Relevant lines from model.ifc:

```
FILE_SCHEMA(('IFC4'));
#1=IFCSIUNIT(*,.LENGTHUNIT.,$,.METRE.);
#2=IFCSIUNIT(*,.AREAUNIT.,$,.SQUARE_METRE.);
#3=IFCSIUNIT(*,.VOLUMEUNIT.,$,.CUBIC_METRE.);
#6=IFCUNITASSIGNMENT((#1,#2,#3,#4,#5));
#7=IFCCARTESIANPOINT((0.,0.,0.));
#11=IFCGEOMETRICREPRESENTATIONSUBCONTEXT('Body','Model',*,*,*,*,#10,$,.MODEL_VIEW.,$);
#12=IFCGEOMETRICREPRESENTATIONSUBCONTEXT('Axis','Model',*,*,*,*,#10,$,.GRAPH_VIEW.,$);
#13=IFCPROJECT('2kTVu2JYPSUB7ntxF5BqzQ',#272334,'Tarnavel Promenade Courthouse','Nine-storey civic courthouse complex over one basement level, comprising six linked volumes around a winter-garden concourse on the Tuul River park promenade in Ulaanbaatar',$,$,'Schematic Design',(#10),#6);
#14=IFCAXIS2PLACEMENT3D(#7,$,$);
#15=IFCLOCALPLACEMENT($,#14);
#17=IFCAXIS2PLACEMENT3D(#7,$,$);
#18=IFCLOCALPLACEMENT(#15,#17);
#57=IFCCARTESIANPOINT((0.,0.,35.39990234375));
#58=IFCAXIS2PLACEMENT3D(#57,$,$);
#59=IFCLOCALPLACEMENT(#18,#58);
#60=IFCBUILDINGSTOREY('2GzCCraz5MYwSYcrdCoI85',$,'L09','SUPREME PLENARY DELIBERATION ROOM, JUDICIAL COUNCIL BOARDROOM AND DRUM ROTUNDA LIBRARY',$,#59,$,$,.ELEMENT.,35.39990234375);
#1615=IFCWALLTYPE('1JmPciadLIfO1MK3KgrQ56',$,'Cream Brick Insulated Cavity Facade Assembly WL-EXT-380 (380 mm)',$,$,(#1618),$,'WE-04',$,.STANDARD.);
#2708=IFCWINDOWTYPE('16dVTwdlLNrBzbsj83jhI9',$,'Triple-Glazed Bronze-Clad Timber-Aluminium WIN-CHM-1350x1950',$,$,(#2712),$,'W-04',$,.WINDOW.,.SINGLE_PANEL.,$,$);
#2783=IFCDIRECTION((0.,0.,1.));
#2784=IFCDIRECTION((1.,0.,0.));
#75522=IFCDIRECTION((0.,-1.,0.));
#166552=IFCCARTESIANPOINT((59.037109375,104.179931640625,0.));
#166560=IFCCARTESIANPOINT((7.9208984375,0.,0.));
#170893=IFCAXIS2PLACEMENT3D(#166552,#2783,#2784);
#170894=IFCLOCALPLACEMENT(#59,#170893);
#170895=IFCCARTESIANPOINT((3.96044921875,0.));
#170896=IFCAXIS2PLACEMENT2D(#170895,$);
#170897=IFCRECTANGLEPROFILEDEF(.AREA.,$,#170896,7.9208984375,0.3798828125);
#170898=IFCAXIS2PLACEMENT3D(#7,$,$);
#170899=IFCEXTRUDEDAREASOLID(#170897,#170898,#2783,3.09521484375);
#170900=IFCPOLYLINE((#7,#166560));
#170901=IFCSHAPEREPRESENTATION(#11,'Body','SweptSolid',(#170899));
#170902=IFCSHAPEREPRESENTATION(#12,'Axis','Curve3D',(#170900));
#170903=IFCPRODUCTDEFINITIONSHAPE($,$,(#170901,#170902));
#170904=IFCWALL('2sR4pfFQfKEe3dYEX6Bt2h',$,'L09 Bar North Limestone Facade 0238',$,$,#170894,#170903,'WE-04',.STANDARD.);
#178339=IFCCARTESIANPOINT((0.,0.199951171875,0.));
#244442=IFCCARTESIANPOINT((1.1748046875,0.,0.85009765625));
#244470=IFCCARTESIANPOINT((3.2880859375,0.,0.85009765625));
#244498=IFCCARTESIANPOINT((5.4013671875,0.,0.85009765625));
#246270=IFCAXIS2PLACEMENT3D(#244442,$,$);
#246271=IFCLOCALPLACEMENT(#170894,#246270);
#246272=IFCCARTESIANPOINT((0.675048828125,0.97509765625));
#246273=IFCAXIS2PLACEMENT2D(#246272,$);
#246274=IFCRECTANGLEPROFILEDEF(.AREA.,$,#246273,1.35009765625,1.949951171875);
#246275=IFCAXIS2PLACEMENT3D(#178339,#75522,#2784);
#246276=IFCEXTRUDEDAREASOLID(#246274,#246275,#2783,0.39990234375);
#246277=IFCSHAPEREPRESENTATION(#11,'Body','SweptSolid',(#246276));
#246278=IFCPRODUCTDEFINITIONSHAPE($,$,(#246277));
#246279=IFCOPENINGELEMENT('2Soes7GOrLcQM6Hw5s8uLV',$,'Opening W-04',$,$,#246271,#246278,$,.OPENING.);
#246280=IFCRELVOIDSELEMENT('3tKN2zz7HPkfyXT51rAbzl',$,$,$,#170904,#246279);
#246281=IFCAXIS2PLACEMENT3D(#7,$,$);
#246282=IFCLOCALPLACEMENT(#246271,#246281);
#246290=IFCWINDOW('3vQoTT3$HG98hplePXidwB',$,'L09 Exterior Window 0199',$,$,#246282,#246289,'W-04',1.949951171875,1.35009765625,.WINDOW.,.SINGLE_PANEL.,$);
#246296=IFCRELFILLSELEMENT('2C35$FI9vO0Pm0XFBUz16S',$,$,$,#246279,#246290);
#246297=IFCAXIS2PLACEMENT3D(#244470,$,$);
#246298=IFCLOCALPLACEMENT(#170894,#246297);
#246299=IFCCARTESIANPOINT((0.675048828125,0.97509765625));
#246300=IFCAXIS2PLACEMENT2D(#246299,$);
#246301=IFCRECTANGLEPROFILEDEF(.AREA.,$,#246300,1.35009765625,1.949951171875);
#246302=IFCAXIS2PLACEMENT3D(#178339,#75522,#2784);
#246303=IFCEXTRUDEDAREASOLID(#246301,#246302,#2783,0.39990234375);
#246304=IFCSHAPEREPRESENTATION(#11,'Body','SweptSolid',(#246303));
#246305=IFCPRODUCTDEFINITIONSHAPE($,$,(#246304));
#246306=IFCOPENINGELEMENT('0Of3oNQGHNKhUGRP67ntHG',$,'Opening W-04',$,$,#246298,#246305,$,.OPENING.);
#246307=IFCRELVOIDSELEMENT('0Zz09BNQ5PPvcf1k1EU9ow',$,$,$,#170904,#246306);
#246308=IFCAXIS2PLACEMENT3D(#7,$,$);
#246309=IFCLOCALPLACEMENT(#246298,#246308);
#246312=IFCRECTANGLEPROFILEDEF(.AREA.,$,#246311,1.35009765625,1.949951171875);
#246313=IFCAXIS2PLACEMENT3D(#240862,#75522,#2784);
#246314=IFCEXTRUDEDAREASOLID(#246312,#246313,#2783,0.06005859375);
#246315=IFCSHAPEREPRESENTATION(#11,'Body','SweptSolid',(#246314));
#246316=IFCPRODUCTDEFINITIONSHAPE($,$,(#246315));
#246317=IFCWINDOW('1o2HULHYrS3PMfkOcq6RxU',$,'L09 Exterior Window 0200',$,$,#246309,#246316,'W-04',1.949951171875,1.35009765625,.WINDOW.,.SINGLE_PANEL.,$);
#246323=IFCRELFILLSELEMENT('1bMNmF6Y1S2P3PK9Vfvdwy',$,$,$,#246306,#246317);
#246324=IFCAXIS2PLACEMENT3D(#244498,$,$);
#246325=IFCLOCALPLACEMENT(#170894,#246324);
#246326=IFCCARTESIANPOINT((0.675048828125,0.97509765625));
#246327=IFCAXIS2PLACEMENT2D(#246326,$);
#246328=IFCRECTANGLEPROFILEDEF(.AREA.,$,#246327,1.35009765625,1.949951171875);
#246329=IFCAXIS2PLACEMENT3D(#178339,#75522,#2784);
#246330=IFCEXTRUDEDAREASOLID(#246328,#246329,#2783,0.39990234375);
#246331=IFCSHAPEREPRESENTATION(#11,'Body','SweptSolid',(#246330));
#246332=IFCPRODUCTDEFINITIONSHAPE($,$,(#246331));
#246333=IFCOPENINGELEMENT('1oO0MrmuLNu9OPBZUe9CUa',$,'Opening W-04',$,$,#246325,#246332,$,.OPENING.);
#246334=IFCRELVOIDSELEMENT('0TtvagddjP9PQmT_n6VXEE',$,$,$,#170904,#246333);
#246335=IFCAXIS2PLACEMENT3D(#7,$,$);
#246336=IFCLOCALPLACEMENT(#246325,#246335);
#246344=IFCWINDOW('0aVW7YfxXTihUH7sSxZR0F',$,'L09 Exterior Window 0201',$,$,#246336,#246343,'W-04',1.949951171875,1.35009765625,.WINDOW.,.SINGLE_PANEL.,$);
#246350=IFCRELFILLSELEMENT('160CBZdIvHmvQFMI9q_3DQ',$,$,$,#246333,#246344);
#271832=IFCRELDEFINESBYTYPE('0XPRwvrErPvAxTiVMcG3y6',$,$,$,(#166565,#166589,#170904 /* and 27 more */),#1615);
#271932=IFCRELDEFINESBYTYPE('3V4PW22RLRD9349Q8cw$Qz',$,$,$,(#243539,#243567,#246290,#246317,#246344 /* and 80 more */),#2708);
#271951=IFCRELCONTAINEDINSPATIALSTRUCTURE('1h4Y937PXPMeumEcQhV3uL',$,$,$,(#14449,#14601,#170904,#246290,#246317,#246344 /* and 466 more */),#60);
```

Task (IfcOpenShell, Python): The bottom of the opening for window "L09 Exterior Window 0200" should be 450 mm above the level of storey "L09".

```python
import numpy as np
import ifcopenshell
import ifcopenshell.api.geometry
import ifcopenshell.geom
import ifcopenshell.util.element
import ifcopenshell.util.placement
import ifcopenshell.util.shape
import ifcopenshell.util.unit

model = ifcopenshell.open("model.ifc")
unit_scale = ifcopenshell.util.unit.calculate_unit_scale(model)

window = model.by_guid("1o2HULHYrS3PMfkOcq6RxU")
opening = window.FillsVoids[0].RelatingOpeningElement
storey = ifcopenshell.util.element.get_container(window, ifc_class="IfcBuildingStorey")
level = ifcopenshell.util.placement.get_local_placement(storey.ObjectPlacement)[2, 3]

# The opening's origin need not be at the sill, so measure its lowest point.
shape = ifcopenshell.geom.create_shape(ifcopenshell.geom.settings(), opening)
bottom = ifcopenshell.util.shape.get_shape_bottom_elevation(shape, shape.geometry) / unit_scale
dz = level + 0.45 / unit_scale - bottom

shift = np.array([0.0, 0.0, dz])
# The window is placed relative to its opening, so it follows when the opening moves.
matrix = ifcopenshell.util.placement.get_local_placement(opening.ObjectPlacement)
matrix[:3, 3] += shift
ifcopenshell.api.geometry.edit_object_placement(
    model, product=opening, matrix=matrix, is_si=False, should_transform_children=True
)

print(f"moved by {dz * unit_scale:+.3f} m")

model.write("model_rev.ifc")
```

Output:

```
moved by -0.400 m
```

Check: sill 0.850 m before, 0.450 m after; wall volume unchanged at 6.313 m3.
